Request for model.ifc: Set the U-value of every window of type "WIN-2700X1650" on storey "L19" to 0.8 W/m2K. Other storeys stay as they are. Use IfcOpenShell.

First a look at what the model holds.

```python
import ifcopenshell
import ifcopenshell.util.element

model = ifcopenshell.open("model.ifc")
print(model.schema)
storey = next(s for s in model.by_type("IfcBuildingStorey") if s.Name == "L19")
windows = [e for e in ifcopenshell.util.element.get_decomposition(storey) if e.is_a("IfcWindow")]
seen = {}
for e in windows:
    element_type = ifcopenshell.util.element.get_type(e)
    key = (element_type.Name if element_type != e and element_type else None, ifcopenshell.util.element.get_pset(e, "Pset_WindowCommon", "ThermalTransmittance"))
    seen[key] = seen.get(key, 0) + 1
for (name, value), count in sorted(seen.items(), key=str):
    print(count, "x", name, "|", value)
```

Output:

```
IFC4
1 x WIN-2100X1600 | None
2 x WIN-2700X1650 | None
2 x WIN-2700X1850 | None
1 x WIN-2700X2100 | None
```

```python
import ifcopenshell
import ifcopenshell.api.pset
import ifcopenshell.util.element

model = ifcopenshell.open("model.ifc")

storey = next(s for s in model.by_type("IfcBuildingStorey") if s.Name == "L19")
windows = [e for e in ifcopenshell.util.element.get_decomposition(storey) if e.is_a("IfcWindow")]

count = 0
for e in windows:
    element_type = ifcopenshell.util.element.get_type(e)
    if element_type in (None, e) or element_type.Name != "WIN-2700X1650":
        continue
    found = ifcopenshell.util.element.get_pset(e, "Pset_WindowCommon", should_inherit=False)
    if found:
        pset = model.by_id(found["id"])
        if len(ifcopenshell.util.element.get_elements_by_pset(pset)) > 1:
            pset = ifcopenshell.api.pset.unshare_pset(model, products=[e], pset=pset)[0]
    else:
        pset = ifcopenshell.api.pset.add_pset(model, product=e, name="Pset_WindowCommon")
    ifcopenshell.api.pset.edit_pset(model, pset=pset, properties={"ThermalTransmittance": 0.8})
    count += 1

print(count, "windows updated")

model.write("model_v2.ifc")
```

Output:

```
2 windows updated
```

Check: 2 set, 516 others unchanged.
